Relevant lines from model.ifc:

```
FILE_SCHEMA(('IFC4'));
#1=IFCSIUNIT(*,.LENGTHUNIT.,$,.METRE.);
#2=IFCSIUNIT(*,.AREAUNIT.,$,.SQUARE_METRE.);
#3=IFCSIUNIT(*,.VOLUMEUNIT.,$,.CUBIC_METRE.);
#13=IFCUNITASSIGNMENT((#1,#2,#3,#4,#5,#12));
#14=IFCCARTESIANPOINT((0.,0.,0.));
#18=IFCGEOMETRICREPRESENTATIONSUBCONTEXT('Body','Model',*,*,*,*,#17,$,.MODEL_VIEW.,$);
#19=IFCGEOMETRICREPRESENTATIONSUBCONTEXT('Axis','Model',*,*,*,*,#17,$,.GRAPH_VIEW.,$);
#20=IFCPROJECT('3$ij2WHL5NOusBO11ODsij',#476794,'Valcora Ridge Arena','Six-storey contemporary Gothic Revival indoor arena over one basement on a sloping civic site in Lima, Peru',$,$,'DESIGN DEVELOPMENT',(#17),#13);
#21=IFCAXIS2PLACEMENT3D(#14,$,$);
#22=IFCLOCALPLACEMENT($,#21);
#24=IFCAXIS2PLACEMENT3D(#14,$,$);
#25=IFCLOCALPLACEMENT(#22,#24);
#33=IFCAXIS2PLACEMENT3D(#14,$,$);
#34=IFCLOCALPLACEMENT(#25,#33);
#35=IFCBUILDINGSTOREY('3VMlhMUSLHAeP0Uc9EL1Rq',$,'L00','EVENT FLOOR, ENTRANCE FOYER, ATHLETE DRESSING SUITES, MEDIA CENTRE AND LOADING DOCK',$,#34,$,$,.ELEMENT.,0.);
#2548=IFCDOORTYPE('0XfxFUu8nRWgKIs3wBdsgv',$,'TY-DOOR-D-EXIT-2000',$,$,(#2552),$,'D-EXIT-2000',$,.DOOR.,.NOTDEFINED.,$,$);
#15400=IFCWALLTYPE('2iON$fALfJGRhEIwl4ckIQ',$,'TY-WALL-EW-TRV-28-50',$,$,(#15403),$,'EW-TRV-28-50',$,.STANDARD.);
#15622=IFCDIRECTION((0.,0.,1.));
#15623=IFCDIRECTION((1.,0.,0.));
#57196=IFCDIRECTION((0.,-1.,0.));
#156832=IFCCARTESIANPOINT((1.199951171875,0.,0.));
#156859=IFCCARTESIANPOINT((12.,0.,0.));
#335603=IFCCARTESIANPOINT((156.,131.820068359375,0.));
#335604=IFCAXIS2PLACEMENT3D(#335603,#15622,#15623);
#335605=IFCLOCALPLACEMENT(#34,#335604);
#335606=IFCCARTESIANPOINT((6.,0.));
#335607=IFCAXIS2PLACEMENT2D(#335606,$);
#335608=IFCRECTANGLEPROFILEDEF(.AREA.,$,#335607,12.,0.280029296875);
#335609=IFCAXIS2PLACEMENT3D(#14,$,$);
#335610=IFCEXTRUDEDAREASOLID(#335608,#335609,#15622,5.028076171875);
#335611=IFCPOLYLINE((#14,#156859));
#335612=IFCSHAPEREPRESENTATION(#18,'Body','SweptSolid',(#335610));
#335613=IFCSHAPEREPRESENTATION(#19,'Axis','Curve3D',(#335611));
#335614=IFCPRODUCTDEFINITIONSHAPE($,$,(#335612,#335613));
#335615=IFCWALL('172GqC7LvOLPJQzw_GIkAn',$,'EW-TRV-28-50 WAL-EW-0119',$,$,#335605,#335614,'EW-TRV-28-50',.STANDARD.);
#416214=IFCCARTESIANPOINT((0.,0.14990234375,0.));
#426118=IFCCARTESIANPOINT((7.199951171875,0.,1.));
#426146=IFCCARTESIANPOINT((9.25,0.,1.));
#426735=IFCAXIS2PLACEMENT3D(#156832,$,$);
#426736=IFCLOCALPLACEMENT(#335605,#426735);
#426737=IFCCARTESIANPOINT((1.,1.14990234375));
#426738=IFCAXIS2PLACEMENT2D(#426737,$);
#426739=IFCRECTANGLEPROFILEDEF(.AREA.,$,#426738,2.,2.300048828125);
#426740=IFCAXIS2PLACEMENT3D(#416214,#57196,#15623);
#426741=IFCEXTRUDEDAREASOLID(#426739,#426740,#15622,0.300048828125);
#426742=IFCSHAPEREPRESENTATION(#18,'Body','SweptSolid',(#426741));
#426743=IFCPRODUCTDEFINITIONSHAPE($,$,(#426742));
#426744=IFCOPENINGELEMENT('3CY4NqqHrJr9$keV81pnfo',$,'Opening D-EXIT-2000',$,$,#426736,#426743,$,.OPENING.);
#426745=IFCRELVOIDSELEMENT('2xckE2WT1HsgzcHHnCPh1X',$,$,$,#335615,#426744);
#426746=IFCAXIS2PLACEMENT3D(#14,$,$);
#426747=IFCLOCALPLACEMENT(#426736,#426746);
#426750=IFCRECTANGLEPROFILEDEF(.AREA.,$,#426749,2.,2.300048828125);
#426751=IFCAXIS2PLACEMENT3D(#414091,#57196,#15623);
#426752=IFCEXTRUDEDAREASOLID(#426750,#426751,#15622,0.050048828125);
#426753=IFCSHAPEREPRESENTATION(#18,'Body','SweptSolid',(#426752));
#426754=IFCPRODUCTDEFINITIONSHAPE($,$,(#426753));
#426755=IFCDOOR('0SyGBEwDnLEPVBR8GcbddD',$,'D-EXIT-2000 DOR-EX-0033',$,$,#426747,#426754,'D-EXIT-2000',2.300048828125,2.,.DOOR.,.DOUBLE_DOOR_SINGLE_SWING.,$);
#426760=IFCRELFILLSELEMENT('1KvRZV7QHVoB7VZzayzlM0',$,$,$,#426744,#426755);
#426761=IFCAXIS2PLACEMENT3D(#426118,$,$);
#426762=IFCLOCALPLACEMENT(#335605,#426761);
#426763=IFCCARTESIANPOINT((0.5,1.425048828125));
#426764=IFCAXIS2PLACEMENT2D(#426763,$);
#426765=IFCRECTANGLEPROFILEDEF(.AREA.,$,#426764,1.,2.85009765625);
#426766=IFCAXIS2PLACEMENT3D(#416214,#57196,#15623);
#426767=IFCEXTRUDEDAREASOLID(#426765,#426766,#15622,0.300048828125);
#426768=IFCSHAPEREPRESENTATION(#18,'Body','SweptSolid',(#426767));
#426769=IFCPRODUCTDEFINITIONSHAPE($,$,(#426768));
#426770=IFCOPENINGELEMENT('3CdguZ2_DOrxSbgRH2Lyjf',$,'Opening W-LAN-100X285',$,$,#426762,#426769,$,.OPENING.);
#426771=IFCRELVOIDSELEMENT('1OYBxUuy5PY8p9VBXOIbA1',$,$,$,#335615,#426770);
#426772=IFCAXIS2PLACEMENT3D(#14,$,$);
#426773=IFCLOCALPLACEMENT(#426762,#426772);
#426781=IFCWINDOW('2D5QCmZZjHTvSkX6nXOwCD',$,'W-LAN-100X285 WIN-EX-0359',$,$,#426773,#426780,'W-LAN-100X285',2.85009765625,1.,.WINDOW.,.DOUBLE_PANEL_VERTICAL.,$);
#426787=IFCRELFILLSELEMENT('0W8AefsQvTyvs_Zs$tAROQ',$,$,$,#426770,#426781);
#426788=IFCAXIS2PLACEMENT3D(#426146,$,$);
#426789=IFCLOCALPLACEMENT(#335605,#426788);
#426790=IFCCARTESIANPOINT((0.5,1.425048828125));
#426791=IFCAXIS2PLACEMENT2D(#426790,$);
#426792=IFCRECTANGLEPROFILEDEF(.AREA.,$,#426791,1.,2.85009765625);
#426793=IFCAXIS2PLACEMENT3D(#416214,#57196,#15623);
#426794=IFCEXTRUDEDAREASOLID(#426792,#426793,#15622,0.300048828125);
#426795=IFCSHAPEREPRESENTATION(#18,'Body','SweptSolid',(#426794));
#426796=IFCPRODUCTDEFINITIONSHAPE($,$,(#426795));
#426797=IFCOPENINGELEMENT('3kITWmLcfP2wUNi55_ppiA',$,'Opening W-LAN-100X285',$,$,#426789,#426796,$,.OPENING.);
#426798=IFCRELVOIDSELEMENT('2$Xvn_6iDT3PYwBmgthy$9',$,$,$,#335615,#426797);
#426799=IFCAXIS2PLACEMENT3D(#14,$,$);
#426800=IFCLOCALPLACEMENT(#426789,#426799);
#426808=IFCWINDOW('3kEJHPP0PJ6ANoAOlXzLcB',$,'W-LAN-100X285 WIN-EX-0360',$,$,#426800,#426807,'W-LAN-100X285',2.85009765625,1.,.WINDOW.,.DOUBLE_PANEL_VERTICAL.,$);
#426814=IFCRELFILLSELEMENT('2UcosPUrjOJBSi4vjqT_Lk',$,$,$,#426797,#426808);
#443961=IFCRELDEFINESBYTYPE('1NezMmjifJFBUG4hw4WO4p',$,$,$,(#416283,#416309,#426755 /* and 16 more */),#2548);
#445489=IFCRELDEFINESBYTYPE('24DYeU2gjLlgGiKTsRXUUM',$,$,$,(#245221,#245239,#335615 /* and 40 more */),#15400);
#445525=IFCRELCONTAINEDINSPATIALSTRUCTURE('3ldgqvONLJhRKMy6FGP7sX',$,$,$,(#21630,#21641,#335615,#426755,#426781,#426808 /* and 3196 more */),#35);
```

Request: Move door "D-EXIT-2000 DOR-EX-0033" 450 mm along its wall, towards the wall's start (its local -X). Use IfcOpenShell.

```python
import ifcopenshell
import ifcopenshell.api.geometry
import ifcopenshell.util.placement

model = ifcopenshell.open("model.ifc")

door = model.by_guid("0SyGBEwDnLEPVBR8GcbddD")
opening = door.FillsVoids[0].RelatingOpeningElement
wall = opening.VoidsElements[0].RelatingBuildingElement

wall_matrix = ifcopenshell.util.placement.get_local_placement(wall.ObjectPlacement)
shift = wall_matrix[:3, 0] * -0.45
before = ifcopenshell.util.placement.get_local_placement(door.ObjectPlacement)[:3, 3].copy()

# The door is placed relative to its opening, so it follows when the opening moves.
matrix = ifcopenshell.util.placement.get_local_placement(opening.ObjectPlacement)
matrix[:3, 3] += shift
ifcopenshell.api.geometry.edit_object_placement(
    model, product=opening, matrix=matrix, is_si=False, should_transform_children=True
)

after = ifcopenshell.util.placement.get_local_placement(door.ObjectPlacement)[:3, 3]
print("door moved by", (after - before).round(3) + 0.0)

model.write("model-out.ifc")
```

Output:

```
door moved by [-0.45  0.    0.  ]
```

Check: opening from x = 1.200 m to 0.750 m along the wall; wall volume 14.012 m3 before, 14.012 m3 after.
